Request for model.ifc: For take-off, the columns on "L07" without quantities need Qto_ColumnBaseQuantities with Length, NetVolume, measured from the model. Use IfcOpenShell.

First a look at what the model holds.

```python
import ifcopenshell
import ifcopenshell.util.element
import ifcopenshell.util.unit

model = ifcopenshell.open("model.ifc")
print(model.schema)
for unit_type in ("LENGTHUNIT", "AREAUNIT", "VOLUMEUNIT"):
    print(unit_type, ifcopenshell.util.unit.calculate_unit_scale(model, unit_type))
storey = next(s for s in model.by_type("IfcBuildingStorey") if s.Name == "L07")
columns = [e for e in ifcopenshell.util.element.get_decomposition(storey) if e.is_a("IfcColumn")]
for e in sorted(columns, key=lambda e: e.id()):
    print(e.id(), e.is_a(), e.Name, list(ifcopenshell.util.element.get_psets(e, qtos_only=True)), sep=" | ")
```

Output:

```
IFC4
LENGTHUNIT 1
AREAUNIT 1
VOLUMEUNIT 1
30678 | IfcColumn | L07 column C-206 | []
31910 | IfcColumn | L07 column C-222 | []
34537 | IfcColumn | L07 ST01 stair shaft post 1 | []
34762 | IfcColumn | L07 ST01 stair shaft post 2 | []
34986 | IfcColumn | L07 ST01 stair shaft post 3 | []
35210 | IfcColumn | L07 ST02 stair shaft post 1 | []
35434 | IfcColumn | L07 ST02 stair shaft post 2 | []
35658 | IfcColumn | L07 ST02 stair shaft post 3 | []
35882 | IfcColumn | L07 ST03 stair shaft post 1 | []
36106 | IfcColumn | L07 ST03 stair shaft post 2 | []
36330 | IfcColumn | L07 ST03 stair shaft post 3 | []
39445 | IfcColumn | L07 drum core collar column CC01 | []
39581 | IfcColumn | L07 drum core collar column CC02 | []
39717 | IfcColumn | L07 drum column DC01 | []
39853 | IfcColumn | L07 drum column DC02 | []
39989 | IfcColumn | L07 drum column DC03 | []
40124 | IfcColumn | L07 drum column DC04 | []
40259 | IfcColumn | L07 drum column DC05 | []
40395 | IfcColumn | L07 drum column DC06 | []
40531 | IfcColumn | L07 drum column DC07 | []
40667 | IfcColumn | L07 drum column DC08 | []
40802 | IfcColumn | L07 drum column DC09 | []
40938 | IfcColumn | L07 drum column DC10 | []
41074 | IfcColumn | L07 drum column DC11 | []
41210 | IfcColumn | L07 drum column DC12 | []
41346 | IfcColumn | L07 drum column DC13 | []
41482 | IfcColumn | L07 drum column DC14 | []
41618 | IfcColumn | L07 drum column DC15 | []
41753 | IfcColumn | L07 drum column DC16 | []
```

```python
import ifcopenshell
import ifcopenshell.api.pset
import ifcopenshell.geom
import ifcopenshell.util.element
import ifcopenshell.util.shape
import ifcopenshell.util.unit

model = ifcopenshell.open("model.ifc")
unit_scale = ifcopenshell.util.unit.calculate_unit_scale(model)
volume_scale = ifcopenshell.util.unit.calculate_unit_scale(model, "VOLUMEUNIT")
settings = ifcopenshell.geom.settings()

storey = next(s for s in model.by_type("IfcBuildingStorey") if s.Name == "L07")
columns = [e for e in ifcopenshell.util.element.get_decomposition(storey) if e.is_a("IfcColumn")]

for e in sorted(columns, key=lambda e: e.id()):
    if ifcopenshell.util.element.get_psets(e, qtos_only=True, should_inherit=False):
        continue
    # Geometry comes back in metres, in the element's own axes.
    shape = ifcopenshell.geom.create_shape(settings, e)
    values = {
        "Length": ifcopenshell.util.shape.get_z(shape.geometry) / unit_scale,
        "NetVolume": ifcopenshell.util.shape.get_volume(shape.geometry) / volume_scale,
    }
    qto = ifcopenshell.api.pset.add_qto(model, product=e, name="Qto_ColumnBaseQuantities")
    ifcopenshell.api.pset.edit_qto(model, qto=qto, properties=values)
    print(e.id(), {k: round(v, 3) for k, v in values.items()})

model.write("model_v2.ifc")
```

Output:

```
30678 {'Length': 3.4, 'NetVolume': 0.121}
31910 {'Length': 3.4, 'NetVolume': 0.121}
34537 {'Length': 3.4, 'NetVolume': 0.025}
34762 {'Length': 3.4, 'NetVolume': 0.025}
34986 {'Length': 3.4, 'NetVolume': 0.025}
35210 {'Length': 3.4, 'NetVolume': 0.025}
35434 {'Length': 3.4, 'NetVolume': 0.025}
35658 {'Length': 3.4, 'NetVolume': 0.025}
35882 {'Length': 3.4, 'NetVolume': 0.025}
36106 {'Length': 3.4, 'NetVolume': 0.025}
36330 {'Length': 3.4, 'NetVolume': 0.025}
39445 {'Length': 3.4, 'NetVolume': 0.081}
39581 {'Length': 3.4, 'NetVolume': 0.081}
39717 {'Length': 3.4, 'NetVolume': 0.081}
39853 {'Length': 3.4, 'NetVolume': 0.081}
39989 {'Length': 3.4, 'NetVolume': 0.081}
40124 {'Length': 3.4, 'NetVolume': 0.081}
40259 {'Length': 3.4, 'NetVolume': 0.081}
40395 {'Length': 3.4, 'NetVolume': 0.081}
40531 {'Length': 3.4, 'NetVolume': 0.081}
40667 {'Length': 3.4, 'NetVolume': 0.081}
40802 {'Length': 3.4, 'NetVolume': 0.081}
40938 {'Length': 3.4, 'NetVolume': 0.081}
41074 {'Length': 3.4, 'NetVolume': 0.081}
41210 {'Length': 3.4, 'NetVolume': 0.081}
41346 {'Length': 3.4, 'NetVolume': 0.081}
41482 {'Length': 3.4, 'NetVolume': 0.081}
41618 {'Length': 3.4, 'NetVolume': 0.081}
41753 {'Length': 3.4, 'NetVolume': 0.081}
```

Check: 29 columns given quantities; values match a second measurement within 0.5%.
